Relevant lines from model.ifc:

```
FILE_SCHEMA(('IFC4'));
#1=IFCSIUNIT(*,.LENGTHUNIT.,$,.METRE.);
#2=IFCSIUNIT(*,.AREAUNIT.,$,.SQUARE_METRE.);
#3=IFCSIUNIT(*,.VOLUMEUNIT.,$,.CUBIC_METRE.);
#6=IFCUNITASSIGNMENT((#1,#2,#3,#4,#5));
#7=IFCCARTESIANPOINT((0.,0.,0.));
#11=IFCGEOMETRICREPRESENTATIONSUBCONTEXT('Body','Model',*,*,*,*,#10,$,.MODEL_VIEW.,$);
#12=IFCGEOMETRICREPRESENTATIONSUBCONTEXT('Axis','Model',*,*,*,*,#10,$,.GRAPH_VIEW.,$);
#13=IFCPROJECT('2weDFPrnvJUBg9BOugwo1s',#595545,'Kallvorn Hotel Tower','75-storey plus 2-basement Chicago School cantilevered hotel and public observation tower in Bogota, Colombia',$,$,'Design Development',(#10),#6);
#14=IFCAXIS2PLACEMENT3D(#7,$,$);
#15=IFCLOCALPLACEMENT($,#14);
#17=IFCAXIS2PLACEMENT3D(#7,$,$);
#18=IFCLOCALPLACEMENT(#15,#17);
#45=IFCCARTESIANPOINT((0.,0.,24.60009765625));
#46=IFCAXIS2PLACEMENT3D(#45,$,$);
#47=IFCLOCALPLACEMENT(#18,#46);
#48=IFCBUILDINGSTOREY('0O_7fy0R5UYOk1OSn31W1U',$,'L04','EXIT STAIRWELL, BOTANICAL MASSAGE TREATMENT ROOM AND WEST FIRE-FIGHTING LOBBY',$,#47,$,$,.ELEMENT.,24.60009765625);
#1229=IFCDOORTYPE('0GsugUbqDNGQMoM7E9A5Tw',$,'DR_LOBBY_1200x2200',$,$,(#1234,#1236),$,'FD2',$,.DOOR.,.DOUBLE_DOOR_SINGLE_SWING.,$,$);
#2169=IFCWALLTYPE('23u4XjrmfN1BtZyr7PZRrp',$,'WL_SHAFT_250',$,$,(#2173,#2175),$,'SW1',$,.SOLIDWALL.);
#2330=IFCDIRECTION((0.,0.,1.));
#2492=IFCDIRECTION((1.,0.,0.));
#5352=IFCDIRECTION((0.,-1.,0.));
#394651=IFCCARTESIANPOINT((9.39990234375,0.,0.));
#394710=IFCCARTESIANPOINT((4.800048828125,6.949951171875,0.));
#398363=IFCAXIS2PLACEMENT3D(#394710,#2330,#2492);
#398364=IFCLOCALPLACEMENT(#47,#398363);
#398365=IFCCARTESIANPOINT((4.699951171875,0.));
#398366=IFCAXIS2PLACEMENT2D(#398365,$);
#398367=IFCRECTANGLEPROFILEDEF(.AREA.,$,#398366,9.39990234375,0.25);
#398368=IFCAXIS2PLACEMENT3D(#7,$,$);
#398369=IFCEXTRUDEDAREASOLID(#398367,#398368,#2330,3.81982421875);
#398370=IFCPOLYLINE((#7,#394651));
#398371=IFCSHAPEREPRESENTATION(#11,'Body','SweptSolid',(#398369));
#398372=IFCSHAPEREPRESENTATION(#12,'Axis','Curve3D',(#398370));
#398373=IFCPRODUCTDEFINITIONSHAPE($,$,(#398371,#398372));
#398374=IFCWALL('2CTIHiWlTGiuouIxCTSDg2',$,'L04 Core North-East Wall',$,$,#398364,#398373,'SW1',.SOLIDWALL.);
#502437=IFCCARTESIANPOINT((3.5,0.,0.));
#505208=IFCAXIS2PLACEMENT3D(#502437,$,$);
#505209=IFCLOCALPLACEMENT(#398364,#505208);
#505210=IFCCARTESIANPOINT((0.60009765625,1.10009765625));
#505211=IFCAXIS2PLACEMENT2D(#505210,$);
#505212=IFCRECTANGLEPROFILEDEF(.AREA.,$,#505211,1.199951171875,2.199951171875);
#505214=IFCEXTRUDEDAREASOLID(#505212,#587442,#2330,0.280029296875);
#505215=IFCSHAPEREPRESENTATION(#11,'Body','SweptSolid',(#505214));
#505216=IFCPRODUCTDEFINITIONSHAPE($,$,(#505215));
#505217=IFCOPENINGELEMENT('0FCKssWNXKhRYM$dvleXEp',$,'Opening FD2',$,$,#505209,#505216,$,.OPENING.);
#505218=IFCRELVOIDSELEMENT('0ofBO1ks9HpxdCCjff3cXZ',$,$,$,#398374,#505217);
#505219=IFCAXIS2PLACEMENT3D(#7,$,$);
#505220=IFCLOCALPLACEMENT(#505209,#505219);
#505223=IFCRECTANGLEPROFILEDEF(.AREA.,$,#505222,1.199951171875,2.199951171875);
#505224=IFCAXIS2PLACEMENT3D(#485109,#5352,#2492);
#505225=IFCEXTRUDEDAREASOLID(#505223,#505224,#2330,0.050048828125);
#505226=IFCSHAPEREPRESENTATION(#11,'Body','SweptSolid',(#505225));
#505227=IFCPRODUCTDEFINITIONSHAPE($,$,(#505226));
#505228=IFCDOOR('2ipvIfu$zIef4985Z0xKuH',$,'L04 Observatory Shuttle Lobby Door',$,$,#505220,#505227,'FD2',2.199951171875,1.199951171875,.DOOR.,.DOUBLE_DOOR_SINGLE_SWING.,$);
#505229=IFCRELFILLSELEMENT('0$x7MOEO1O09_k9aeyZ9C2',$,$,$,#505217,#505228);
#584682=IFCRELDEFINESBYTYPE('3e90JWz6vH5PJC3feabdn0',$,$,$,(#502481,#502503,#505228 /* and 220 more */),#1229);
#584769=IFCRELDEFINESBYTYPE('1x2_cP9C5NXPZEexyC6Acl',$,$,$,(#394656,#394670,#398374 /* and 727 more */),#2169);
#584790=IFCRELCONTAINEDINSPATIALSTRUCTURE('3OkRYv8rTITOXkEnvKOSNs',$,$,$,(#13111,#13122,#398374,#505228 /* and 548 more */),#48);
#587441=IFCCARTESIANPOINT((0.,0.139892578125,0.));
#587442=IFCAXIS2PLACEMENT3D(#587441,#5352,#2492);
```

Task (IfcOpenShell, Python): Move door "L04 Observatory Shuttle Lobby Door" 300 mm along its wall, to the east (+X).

```python
import ifcopenshell
import ifcopenshell.api.geometry
import ifcopenshell.util.placement
import ifcopenshell.util.unit

model = ifcopenshell.open("model.ifc")
unit_scale = ifcopenshell.util.unit.calculate_unit_scale(model)

door = model.by_id(505228)
opening = door.FillsVoids[0].RelatingOpeningElement
wall = opening.VoidsElements[0].RelatingBuildingElement

wall_matrix = ifcopenshell.util.placement.get_local_placement(wall.ObjectPlacement)
shift = wall_matrix[:3, 0] * 0.3 / unit_scale
before = ifcopenshell.util.placement.get_local_placement(door.ObjectPlacement)[:3, 3].copy()

# The door is placed relative to its opening, so it follows when the opening moves.
matrix = ifcopenshell.util.placement.get_local_placement(opening.ObjectPlacement)
matrix[:3, 3] += shift
ifcopenshell.api.geometry.edit_object_placement(
    model, product=opening, matrix=matrix, is_si=False, should_transform_children=True
)

after = ifcopenshell.util.placement.get_local_placement(door.ObjectPlacement)[:3, 3]
print("door moved by", (after - before).round(3) + 0.0)

model.write("model-out.ifc")
```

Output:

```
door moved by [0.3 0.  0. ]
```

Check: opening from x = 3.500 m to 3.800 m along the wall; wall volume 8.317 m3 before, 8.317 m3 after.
